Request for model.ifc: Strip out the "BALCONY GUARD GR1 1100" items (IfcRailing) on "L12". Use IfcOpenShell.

First a look at what the model holds.

```python
import ifcopenshell
import ifcopenshell.util.element

model = ifcopenshell.open("model.ifc")
print(model.schema)
storey = next(s for s in model.by_type("IfcBuildingStorey") if s.Name == "L12")
railings = [e for e in ifcopenshell.util.element.get_decomposition(storey) if e.is_a("IfcRailing")]
seen = {}
for e in railings:
    element_type = ifcopenshell.util.element.get_type(e)
    name = element_type.Name if element_type not in (None, e) else None
    seen[name] = seen.get(name, 0) + 1
for name, count in sorted(seen.items(), key=str):
    print(count, "x", name)
```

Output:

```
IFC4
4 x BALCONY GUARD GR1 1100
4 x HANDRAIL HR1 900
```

```python
import ifcopenshell
import ifcopenshell.api.root
import ifcopenshell.util.element

model = ifcopenshell.open("model.ifc")

storey = next(s for s in model.by_type("IfcBuildingStorey") if s.Name == "L12")
railings = [e for e in ifcopenshell.util.element.get_decomposition(storey) if e.is_a("IfcRailing")]
targets = [e for e in railings if (t := ifcopenshell.util.element.get_type(e)) not in (None, e) and t.Name == "BALCONY GUARD GR1 1100"]

for e in targets:
    ifcopenshell.api.root.remove_product(model, product=e)
print(len(targets), "removed")

model.write("model_v2.ifc")
```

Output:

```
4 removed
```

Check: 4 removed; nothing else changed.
